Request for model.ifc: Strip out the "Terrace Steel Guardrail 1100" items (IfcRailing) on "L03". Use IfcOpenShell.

First a look at what the model holds.

```python
import ifcopenshell
import ifcopenshell.util.element

model = ifcopenshell.open("model.ifc")
print(model.schema)
storey = next(s for s in model.by_type("IfcBuildingStorey") if s.Name == "L03")
railings = [e for e in ifcopenshell.util.element.get_decomposition(storey) if e.is_a("IfcRailing")]
seen = {}
for e in railings:
    element_type = ifcopenshell.util.element.get_type(e)
    name = element_type.Name if element_type not in (None, e) else None
    seen[name] = seen.get(name, 0) + 1
for name, count in sorted(seen.items(), key=str):
    print(count, "x", name)
```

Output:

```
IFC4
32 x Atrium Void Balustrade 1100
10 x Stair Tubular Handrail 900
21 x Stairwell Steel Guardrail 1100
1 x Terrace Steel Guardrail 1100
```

```python
import ifcopenshell
import ifcopenshell.api.root
import ifcopenshell.util.element

model = ifcopenshell.open("model.ifc")

storey = next(s for s in model.by_type("IfcBuildingStorey") if s.Name == "L03")
railings = [e for e in ifcopenshell.util.element.get_decomposition(storey) if e.is_a("IfcRailing")]
targets = [e for e in railings if (t := ifcopenshell.util.element.get_type(e)) not in (None, e) and t.Name == "Terrace Steel Guardrail 1100"]

for e in targets:
    ifcopenshell.api.root.remove_product(model, product=e)
print(len(targets), "removed")

model.write("model-out.ifc")
```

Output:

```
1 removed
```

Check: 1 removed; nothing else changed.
